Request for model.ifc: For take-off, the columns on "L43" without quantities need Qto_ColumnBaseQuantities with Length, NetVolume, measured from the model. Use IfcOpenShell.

First a look at what the model holds.

```python
import ifcopenshell
import ifcopenshell.util.element
import ifcopenshell.util.unit

model = ifcopenshell.open("model.ifc")
print(model.schema)
for unit_type in ("LENGTHUNIT", "AREAUNIT", "VOLUMEUNIT"):
    print(unit_type, ifcopenshell.util.unit.calculate_unit_scale(model, unit_type))
storey = next(s for s in model.by_type("IfcBuildingStorey") if s.Name == "L43")
columns = [e for e in ifcopenshell.util.element.get_decomposition(storey) if e.is_a("IfcColumn")]
for e in sorted(columns, key=lambda e: e.id()):
    print(e.id(), e.is_a(), e.Name, list(ifcopenshell.util.element.get_psets(e, qtos_only=True)), sep=" | ")
```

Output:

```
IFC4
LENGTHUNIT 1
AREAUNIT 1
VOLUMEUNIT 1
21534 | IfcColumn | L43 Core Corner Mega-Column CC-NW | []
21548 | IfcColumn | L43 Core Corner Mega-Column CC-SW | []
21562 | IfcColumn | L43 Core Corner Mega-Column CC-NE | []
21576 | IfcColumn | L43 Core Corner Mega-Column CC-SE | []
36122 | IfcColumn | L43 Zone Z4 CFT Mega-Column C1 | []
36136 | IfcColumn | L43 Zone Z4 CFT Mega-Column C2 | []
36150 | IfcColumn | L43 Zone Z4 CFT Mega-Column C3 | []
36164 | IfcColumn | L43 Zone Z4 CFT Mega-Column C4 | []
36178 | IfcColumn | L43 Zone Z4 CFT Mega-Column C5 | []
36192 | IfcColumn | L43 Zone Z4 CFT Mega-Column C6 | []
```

```python
import ifcopenshell
import ifcopenshell.api.pset
import ifcopenshell.geom
import ifcopenshell.util.element
import ifcopenshell.util.shape
import ifcopenshell.util.unit

model = ifcopenshell.open("model.ifc")
unit_scale = ifcopenshell.util.unit.calculate_unit_scale(model)
volume_scale = ifcopenshell.util.unit.calculate_unit_scale(model, "VOLUMEUNIT")
settings = ifcopenshell.geom.settings()

storey = next(s for s in model.by_type("IfcBuildingStorey") if s.Name == "L43")
columns = [e for e in ifcopenshell.util.element.get_decomposition(storey) if e.is_a("IfcColumn")]

for e in sorted(columns, key=lambda e: e.id()):
    if ifcopenshell.util.element.get_psets(e, qtos_only=True, should_inherit=False):
        continue
    # Geometry comes back in metres, in the element's own axes.
    shape = ifcopenshell.geom.create_shape(settings, e)
    values = {
        "Length": ifcopenshell.util.shape.get_z(shape.geometry) / unit_scale,
        "NetVolume": ifcopenshell.util.shape.get_volume(shape.geometry) / volume_scale,
    }
    qto = ifcopenshell.api.pset.add_qto(model, product=e, name="Qto_ColumnBaseQuantities")
    ifcopenshell.api.pset.edit_qto(model, qto=qto, properties=values)
    print(e.id(), {k: round(v, 3) for k, v in values.items()})

model.write("model_rev.ifc")
```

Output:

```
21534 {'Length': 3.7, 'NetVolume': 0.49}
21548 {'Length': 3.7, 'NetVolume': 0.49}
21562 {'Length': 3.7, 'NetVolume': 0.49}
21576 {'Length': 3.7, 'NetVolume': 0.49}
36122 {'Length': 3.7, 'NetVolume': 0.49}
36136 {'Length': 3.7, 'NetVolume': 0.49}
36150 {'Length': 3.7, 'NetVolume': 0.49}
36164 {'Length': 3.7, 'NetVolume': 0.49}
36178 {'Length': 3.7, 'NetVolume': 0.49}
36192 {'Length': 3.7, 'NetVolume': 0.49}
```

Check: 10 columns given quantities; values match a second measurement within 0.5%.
